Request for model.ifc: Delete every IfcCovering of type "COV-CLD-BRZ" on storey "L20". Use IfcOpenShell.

First a look at what the model holds.

```python
import ifcopenshell
import ifcopenshell.util.element

model = ifcopenshell.open("model.ifc")
print(model.schema)
storey = next(s for s in model.by_type("IfcBuildingStorey") if s.Name == "L20")
coverings = [e for e in ifcopenshell.util.element.get_decomposition(storey) if e.is_a("IfcCovering")]
seen = {}
for e in coverings:
    element_type = ifcopenshell.util.element.get_type(e)
    name = element_type.Name if element_type not in (None, e) else None
    seen[name] = seen.get(name, 0) + 1
for name, count in sorted(seen.items(), key=str):
    print(count, "x", name)
```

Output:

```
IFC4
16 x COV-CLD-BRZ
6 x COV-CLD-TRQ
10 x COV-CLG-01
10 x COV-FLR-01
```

```python
import ifcopenshell
import ifcopenshell.api.root
import ifcopenshell.util.element

model = ifcopenshell.open("model.ifc")

storey = next(s for s in model.by_type("IfcBuildingStorey") if s.Name == "L20")
coverings = [e for e in ifcopenshell.util.element.get_decomposition(storey) if e.is_a("IfcCovering")]
targets = [e for e in coverings if (t := ifcopenshell.util.element.get_type(e)) not in (None, e) and t.Name == "COV-CLD-BRZ"]

for e in targets:
    ifcopenshell.api.root.remove_product(model, product=e)
print(len(targets), "removed")

model.write("model_updated.ifc")
```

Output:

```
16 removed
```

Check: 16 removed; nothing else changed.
